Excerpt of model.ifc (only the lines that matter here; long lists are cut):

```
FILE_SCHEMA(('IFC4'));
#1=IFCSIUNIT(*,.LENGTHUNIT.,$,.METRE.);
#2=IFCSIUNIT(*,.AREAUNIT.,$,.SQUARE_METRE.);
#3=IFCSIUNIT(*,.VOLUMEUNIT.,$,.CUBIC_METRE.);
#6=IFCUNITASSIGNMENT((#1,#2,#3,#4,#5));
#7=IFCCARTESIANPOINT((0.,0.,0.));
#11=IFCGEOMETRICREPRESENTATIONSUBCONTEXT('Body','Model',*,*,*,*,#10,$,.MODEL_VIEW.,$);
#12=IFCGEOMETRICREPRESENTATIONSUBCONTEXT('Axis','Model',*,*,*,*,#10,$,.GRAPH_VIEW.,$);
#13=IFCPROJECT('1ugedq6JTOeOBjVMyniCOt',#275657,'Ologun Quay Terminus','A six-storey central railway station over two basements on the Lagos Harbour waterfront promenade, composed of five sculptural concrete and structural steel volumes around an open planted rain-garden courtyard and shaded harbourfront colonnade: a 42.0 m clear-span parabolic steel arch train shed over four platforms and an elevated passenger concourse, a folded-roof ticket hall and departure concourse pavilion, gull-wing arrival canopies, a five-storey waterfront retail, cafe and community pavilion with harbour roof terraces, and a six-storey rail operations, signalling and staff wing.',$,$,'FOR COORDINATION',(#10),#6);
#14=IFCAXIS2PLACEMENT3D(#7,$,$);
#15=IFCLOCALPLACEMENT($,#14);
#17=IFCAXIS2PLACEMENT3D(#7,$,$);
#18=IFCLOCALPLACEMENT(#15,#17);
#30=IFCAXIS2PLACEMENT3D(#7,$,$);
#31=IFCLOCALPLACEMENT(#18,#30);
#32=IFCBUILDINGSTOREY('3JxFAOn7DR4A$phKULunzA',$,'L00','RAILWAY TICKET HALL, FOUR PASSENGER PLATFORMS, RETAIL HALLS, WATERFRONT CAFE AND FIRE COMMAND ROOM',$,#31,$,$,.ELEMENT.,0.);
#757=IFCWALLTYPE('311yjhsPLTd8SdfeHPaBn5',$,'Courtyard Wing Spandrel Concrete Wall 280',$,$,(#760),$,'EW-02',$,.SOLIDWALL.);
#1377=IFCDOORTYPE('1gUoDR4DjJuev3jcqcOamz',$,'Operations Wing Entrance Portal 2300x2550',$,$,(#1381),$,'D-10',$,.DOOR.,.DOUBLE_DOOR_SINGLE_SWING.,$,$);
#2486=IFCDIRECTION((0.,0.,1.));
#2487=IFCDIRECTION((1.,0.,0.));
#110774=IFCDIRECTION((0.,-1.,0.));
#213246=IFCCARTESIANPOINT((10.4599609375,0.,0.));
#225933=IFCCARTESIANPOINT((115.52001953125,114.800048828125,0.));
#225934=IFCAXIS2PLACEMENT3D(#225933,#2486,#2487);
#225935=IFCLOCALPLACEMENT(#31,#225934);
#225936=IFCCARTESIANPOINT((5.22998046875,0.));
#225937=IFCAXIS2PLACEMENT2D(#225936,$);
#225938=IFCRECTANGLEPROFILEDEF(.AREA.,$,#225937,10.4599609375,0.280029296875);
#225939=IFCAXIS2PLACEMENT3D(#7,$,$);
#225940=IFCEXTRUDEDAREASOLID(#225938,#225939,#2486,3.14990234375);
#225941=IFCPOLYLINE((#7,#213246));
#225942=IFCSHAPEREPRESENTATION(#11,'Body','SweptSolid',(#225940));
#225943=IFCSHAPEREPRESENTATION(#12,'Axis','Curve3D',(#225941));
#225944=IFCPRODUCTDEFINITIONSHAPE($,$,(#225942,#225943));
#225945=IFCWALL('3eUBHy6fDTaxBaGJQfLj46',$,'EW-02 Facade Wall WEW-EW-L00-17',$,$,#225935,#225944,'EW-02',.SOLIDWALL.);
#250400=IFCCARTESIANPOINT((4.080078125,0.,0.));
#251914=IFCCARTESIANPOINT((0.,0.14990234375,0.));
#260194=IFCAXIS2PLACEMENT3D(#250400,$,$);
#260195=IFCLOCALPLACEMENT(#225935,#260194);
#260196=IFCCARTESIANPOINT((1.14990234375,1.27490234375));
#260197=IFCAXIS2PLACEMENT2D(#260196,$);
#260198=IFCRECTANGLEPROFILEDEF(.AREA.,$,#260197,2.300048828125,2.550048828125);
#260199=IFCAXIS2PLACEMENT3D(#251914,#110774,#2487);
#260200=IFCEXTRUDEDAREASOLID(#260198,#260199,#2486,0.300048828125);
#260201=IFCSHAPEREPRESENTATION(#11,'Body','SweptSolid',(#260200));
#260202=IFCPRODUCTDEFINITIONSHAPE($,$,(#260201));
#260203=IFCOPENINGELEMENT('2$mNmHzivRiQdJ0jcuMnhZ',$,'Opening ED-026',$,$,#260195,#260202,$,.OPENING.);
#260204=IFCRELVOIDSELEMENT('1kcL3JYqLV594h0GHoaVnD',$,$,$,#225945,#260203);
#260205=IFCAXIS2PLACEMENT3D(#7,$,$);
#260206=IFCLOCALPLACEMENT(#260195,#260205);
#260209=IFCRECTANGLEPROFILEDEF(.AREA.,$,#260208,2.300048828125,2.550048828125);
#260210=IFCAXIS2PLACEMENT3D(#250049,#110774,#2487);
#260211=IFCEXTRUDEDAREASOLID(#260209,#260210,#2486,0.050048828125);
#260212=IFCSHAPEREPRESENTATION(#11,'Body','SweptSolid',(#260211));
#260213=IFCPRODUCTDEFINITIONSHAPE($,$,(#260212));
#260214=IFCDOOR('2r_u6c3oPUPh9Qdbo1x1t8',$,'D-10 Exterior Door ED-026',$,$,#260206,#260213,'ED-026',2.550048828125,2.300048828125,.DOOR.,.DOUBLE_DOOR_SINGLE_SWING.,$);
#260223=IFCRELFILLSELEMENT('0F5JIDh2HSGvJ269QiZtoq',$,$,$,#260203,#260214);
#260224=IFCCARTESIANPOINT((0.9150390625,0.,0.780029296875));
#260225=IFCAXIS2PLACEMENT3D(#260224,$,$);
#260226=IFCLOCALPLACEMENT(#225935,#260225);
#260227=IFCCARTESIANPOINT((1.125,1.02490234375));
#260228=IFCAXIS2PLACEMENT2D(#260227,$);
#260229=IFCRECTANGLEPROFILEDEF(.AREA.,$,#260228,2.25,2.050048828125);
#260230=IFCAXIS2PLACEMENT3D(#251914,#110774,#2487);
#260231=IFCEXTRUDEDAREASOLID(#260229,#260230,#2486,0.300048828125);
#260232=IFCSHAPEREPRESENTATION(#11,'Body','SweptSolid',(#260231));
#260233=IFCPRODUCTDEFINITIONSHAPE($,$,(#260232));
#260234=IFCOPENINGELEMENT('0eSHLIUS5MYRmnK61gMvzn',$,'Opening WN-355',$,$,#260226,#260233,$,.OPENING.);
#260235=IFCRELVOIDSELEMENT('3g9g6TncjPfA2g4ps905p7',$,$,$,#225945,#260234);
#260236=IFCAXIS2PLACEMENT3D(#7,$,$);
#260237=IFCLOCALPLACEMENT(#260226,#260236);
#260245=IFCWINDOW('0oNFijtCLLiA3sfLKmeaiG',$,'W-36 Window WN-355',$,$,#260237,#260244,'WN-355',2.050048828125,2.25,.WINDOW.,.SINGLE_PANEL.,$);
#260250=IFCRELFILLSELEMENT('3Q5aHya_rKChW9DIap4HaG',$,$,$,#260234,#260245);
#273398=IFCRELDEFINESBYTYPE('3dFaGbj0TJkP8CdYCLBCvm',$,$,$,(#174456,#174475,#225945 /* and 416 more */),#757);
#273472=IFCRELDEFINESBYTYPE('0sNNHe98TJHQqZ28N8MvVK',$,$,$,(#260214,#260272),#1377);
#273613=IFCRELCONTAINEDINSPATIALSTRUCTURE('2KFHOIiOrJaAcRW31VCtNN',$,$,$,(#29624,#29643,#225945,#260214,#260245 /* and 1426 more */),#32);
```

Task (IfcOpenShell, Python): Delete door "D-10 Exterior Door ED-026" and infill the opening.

```python
import ifcopenshell
import ifcopenshell.api.feature
import ifcopenshell.api.root
import ifcopenshell.geom
import ifcopenshell.util.shape

model = ifcopenshell.open("model.ifc")
settings = ifcopenshell.geom.settings()


def volume(element):
    """Net volume in cubic metres, openings subtracted."""
    shape = ifcopenshell.geom.create_shape(settings, element)
    return ifcopenshell.util.shape.get_volume(shape.geometry)


door = model.by_guid("2r_u6c3oPUPh9Qdbo1x1t8")
opening = door.FillsVoids[0].RelatingOpeningElement
wall = opening.VoidsElements[0].RelatingBuildingElement
before = volume(wall)

ifcopenshell.api.root.remove_product(model, product=door)
ifcopenshell.api.feature.remove_feature(model, feature=opening)

after = volume(wall)

print(f"wall volume {before:.3f} -> {after:.3f} m3")

model.write("model-out.ifc")
```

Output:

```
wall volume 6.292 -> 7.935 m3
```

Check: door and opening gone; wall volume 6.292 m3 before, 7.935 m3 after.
